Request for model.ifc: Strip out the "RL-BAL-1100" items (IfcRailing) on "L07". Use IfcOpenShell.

First a look at what the model holds.

```python
import ifcopenshell
import ifcopenshell.util.element

model = ifcopenshell.open("model.ifc")
print(model.schema)
storey = next(s for s in model.by_type("IfcBuildingStorey") if s.Name == "L07")
railings = [e for e in ifcopenshell.util.element.get_decomposition(storey) if e.is_a("IfcRailing")]
seen = {}
for e in railings:
    element_type = ifcopenshell.util.element.get_type(e)
    name = element_type.Name if element_type not in (None, e) else None
    seen[name] = seen.get(name, 0) + 1
for name, count in sorted(seen.items(), key=str):
    print(count, "x", name)
```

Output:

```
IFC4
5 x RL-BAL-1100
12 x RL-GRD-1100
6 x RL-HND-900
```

```python
import ifcopenshell
import ifcopenshell.api.root
import ifcopenshell.util.element

model = ifcopenshell.open("model.ifc")

storey = next(s for s in model.by_type("IfcBuildingStorey") if s.Name == "L07")
railings = [e for e in ifcopenshell.util.element.get_decomposition(storey) if e.is_a("IfcRailing")]
targets = [e for e in railings if (t := ifcopenshell.util.element.get_type(e)) not in (None, e) and t.Name == "RL-BAL-1100"]

for e in targets:
    ifcopenshell.api.root.remove_product(model, product=e)
print(len(targets), "removed")

model.write("model_edited.ifc")
```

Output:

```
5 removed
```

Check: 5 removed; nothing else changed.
